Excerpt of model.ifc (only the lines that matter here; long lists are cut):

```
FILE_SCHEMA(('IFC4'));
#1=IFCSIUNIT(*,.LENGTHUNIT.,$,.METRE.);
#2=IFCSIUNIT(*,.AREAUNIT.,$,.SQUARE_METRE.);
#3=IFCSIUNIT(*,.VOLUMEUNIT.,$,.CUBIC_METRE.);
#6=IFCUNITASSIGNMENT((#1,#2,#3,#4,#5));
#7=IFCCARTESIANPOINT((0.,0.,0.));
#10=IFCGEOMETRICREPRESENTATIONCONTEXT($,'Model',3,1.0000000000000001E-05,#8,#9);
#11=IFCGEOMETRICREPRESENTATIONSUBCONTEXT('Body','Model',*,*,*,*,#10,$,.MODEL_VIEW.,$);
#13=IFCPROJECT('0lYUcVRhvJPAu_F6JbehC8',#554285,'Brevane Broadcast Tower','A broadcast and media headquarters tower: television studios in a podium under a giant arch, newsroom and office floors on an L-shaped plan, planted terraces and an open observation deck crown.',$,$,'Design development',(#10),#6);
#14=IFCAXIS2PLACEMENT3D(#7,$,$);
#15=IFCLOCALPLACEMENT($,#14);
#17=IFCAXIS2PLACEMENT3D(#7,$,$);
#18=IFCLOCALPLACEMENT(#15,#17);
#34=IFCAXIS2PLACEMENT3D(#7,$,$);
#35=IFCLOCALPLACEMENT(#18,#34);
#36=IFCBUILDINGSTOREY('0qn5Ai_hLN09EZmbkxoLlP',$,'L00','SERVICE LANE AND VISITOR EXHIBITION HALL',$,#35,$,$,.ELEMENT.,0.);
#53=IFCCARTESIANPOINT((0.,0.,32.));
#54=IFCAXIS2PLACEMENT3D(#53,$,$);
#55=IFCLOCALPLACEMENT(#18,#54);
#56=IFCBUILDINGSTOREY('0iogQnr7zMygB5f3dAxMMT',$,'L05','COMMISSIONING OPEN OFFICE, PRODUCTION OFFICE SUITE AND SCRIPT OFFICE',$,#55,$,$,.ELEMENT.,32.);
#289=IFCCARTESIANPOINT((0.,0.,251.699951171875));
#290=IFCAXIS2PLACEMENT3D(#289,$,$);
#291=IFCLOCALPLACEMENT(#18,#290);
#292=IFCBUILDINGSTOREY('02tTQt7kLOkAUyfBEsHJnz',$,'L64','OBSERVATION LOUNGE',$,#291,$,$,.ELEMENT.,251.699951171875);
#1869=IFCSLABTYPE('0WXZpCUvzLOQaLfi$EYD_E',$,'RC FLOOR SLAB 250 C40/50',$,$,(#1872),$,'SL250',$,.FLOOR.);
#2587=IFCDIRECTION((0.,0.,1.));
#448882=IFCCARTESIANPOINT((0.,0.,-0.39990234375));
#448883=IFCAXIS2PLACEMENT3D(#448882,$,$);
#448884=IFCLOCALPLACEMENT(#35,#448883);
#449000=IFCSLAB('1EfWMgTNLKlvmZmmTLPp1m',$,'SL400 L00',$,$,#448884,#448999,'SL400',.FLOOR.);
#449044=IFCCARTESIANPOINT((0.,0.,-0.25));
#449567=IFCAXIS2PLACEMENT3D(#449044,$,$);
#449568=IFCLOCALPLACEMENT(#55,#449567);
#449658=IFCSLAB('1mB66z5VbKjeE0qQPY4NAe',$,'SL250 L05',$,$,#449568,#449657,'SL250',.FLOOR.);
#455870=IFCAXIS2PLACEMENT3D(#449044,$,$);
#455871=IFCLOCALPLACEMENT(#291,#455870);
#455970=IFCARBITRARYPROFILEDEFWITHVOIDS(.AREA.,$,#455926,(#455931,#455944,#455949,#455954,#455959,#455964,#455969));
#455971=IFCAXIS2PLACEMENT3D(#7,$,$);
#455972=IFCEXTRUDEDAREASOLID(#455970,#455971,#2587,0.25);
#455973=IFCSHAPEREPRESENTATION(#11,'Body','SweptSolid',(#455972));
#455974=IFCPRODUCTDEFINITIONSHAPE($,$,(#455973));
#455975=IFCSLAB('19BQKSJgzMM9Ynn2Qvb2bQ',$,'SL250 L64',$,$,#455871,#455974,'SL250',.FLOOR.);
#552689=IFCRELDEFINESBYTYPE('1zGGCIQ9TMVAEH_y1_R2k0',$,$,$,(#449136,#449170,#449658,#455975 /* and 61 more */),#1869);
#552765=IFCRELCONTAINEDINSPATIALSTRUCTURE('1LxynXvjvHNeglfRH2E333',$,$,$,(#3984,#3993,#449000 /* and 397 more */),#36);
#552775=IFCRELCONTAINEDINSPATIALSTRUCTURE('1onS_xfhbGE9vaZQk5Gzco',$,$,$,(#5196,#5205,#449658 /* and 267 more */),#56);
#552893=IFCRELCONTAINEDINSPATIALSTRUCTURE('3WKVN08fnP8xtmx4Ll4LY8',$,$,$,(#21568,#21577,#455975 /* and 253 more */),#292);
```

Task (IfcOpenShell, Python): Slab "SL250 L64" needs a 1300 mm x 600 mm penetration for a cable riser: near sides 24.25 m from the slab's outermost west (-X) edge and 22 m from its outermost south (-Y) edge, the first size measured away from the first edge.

```python
import numpy as np
import ifcopenshell
import ifcopenshell.api.feature
import ifcopenshell.api.geometry
import ifcopenshell.api.root
import ifcopenshell.geom
import ifcopenshell.util.placement
import ifcopenshell.util.representation
import ifcopenshell.util.shape
import ifcopenshell.util.unit

model = ifcopenshell.open("model.ifc")
unit_scale = ifcopenshell.util.unit.calculate_unit_scale(model)
settings = ifcopenshell.geom.settings()


def volume(element):
    """Net volume in cubic metres, openings subtracted."""
    shape = ifcopenshell.geom.create_shape(settings, element)
    return ifcopenshell.util.shape.get_volume(shape.geometry)


slab = model.by_id(455975)
before = volume(slab)

# Extent in the slab's own axes, in metres. The edges named are its -X and -Y sides.
slab_shape = ifcopenshell.geom.create_shape(settings, slab)
vertices = ifcopenshell.util.shape.get_vertices(slab_shape.geometry)
x_min, y_min, bottom = vertices.min(axis=0)
top = vertices[:, 2].max()

opening = ifcopenshell.api.root.create_entity(model, ifc_class="IfcOpeningElement", name="Cable riser opening", predefined_type="OPENING")
context = ifcopenshell.util.representation.get_context(model, "Model", "Body", "MODEL_VIEW")
width, depth = 1.3, 0.6
outline = [(0.0, 0.0), (width, 0.0), (width, depth), (0.0, depth), (0.0, 0.0)]
# Overshoot both faces by 50 mm so the cut is clean.
shape = ifcopenshell.api.geometry.add_slab_representation(
    model, context=context, depth=top - bottom + 0.1, polyline=outline
)
ifcopenshell.api.geometry.assign_representation(model, product=opening, representation=shape)

matrix = ifcopenshell.util.placement.get_local_placement(slab.ObjectPlacement)
matrix[:, 3] = matrix @ np.append(np.array([x_min + 24.25, y_min + 22, bottom - 0.05]) / unit_scale, 1.0)
ifcopenshell.api.geometry.edit_object_placement(model, product=opening, matrix=matrix, is_si=False)
ifcopenshell.api.feature.add_feature(model, feature=opening, element=slab)

after = volume(slab)

print(f"slab volume {before:.3f} -> {after:.3f} m3")

model.write("model_rev.ifc")
```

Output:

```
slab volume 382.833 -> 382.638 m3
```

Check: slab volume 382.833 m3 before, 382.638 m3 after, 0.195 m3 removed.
